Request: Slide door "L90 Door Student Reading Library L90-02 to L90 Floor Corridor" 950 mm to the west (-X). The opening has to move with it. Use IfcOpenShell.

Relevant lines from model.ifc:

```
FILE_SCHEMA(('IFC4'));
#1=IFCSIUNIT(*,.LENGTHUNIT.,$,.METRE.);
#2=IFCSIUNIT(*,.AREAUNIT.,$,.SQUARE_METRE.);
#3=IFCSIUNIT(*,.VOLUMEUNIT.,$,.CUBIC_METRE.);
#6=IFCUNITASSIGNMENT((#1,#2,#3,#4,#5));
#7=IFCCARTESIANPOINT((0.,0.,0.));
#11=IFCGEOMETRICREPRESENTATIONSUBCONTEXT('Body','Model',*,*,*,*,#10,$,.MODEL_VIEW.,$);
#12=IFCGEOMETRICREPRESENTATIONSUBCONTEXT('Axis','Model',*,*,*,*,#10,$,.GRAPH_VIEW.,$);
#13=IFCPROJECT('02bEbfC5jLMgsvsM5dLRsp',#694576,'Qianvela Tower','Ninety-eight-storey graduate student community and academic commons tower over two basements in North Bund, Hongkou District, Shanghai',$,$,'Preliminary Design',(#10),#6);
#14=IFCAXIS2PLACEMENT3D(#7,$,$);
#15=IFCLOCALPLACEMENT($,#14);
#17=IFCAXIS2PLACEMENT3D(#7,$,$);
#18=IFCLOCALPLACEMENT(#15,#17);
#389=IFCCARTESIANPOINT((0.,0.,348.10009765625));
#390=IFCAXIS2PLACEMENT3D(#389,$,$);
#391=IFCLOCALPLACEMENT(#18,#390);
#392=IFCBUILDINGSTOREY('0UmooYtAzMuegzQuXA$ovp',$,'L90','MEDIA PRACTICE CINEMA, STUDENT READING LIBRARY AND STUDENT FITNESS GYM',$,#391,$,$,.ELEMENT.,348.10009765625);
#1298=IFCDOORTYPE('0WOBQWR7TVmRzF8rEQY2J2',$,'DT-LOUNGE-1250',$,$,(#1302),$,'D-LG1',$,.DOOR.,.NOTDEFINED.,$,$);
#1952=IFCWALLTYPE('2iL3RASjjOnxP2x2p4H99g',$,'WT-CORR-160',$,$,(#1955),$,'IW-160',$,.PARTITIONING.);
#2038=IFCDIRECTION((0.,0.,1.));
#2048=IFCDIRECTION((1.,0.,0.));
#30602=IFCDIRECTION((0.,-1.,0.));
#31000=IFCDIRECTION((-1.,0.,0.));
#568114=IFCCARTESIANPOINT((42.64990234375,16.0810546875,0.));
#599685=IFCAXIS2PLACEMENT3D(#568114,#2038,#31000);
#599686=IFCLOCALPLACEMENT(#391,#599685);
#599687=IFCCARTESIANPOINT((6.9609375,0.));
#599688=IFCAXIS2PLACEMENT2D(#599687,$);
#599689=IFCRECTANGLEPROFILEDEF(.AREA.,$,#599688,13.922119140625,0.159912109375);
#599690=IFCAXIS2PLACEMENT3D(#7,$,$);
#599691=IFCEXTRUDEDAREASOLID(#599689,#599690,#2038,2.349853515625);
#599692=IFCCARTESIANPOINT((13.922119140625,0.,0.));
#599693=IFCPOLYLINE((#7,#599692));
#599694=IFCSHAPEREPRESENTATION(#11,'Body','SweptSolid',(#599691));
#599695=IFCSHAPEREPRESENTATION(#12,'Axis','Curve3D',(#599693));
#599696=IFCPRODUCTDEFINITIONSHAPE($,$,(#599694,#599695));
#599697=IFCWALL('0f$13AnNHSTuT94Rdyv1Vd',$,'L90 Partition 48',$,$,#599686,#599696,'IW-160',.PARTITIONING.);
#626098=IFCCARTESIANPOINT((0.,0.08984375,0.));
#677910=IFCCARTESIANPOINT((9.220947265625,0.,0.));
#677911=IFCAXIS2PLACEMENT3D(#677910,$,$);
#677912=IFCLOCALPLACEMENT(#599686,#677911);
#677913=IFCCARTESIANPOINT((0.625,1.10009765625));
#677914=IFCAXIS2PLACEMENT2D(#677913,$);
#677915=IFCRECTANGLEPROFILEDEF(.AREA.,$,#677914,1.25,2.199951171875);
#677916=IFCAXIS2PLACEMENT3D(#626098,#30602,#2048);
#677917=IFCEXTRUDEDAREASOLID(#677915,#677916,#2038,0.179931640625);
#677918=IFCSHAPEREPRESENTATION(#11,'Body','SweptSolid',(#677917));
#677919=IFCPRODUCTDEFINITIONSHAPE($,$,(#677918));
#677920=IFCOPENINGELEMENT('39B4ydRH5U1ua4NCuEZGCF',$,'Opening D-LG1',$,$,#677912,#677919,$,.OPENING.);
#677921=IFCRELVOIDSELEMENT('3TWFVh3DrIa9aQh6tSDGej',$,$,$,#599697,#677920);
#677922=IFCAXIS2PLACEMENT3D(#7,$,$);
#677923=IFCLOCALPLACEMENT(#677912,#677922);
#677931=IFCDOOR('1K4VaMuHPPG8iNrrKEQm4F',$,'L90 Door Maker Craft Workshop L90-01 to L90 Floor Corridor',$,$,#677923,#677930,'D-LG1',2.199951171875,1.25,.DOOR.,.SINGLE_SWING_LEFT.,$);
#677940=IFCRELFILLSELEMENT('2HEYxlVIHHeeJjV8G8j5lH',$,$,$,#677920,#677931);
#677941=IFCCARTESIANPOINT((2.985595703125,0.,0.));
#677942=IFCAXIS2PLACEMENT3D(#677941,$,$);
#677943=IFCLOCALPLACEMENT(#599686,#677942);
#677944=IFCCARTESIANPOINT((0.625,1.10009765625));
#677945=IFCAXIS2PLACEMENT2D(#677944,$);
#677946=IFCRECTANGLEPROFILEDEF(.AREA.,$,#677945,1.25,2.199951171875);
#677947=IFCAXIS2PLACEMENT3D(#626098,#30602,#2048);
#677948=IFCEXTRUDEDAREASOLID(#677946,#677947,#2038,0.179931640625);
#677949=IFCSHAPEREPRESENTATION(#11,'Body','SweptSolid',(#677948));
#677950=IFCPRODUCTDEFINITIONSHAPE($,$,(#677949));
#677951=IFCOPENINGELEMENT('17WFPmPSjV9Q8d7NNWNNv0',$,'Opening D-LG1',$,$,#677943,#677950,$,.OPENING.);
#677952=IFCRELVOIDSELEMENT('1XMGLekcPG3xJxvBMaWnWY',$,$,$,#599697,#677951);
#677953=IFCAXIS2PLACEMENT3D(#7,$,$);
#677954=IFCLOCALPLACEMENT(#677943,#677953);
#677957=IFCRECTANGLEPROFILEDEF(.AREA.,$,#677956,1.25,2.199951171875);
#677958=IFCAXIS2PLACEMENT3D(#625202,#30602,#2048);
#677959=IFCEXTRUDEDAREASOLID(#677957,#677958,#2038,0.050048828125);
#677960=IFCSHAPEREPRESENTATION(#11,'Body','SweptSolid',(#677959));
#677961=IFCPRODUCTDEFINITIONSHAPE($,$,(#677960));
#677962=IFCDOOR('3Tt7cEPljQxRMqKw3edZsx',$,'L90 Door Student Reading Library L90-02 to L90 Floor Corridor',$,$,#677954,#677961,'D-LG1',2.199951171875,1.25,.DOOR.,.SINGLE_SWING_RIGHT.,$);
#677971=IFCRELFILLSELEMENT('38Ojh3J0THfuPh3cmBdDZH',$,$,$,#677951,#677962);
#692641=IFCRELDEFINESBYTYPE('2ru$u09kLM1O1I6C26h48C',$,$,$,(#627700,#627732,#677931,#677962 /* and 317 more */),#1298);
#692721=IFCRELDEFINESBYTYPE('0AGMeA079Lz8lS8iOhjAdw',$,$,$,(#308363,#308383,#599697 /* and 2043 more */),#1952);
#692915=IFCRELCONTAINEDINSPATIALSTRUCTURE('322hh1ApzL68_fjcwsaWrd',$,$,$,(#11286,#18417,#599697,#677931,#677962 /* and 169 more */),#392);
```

```python
import ifcopenshell
import ifcopenshell.api.geometry
import ifcopenshell.util.placement
import ifcopenshell.util.unit

model = ifcopenshell.open("model.ifc")
unit_scale = ifcopenshell.util.unit.calculate_unit_scale(model)

door = model.by_id(677962)
opening = door.FillsVoids[0].RelatingOpeningElement
wall = opening.VoidsElements[0].RelatingBuildingElement

wall_matrix = ifcopenshell.util.placement.get_local_placement(wall.ObjectPlacement)
shift = wall_matrix[:3, 0] * 0.95 / unit_scale
before = ifcopenshell.util.placement.get_local_placement(door.ObjectPlacement)[:3, 3].copy()

# The door is placed relative to its opening, so it follows when the opening moves.
matrix = ifcopenshell.util.placement.get_local_placement(opening.ObjectPlacement)
matrix[:3, 3] += shift
ifcopenshell.api.geometry.edit_object_placement(
    model, product=opening, matrix=matrix, is_si=False, should_transform_children=True
)

after = ifcopenshell.util.placement.get_local_placement(door.ObjectPlacement)[:3, 3]
print("door moved by", (after - before).round(3) + 0.0)

model.write("model_edited.ifc")
```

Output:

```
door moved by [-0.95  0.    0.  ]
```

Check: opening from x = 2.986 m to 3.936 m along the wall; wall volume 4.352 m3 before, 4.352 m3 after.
